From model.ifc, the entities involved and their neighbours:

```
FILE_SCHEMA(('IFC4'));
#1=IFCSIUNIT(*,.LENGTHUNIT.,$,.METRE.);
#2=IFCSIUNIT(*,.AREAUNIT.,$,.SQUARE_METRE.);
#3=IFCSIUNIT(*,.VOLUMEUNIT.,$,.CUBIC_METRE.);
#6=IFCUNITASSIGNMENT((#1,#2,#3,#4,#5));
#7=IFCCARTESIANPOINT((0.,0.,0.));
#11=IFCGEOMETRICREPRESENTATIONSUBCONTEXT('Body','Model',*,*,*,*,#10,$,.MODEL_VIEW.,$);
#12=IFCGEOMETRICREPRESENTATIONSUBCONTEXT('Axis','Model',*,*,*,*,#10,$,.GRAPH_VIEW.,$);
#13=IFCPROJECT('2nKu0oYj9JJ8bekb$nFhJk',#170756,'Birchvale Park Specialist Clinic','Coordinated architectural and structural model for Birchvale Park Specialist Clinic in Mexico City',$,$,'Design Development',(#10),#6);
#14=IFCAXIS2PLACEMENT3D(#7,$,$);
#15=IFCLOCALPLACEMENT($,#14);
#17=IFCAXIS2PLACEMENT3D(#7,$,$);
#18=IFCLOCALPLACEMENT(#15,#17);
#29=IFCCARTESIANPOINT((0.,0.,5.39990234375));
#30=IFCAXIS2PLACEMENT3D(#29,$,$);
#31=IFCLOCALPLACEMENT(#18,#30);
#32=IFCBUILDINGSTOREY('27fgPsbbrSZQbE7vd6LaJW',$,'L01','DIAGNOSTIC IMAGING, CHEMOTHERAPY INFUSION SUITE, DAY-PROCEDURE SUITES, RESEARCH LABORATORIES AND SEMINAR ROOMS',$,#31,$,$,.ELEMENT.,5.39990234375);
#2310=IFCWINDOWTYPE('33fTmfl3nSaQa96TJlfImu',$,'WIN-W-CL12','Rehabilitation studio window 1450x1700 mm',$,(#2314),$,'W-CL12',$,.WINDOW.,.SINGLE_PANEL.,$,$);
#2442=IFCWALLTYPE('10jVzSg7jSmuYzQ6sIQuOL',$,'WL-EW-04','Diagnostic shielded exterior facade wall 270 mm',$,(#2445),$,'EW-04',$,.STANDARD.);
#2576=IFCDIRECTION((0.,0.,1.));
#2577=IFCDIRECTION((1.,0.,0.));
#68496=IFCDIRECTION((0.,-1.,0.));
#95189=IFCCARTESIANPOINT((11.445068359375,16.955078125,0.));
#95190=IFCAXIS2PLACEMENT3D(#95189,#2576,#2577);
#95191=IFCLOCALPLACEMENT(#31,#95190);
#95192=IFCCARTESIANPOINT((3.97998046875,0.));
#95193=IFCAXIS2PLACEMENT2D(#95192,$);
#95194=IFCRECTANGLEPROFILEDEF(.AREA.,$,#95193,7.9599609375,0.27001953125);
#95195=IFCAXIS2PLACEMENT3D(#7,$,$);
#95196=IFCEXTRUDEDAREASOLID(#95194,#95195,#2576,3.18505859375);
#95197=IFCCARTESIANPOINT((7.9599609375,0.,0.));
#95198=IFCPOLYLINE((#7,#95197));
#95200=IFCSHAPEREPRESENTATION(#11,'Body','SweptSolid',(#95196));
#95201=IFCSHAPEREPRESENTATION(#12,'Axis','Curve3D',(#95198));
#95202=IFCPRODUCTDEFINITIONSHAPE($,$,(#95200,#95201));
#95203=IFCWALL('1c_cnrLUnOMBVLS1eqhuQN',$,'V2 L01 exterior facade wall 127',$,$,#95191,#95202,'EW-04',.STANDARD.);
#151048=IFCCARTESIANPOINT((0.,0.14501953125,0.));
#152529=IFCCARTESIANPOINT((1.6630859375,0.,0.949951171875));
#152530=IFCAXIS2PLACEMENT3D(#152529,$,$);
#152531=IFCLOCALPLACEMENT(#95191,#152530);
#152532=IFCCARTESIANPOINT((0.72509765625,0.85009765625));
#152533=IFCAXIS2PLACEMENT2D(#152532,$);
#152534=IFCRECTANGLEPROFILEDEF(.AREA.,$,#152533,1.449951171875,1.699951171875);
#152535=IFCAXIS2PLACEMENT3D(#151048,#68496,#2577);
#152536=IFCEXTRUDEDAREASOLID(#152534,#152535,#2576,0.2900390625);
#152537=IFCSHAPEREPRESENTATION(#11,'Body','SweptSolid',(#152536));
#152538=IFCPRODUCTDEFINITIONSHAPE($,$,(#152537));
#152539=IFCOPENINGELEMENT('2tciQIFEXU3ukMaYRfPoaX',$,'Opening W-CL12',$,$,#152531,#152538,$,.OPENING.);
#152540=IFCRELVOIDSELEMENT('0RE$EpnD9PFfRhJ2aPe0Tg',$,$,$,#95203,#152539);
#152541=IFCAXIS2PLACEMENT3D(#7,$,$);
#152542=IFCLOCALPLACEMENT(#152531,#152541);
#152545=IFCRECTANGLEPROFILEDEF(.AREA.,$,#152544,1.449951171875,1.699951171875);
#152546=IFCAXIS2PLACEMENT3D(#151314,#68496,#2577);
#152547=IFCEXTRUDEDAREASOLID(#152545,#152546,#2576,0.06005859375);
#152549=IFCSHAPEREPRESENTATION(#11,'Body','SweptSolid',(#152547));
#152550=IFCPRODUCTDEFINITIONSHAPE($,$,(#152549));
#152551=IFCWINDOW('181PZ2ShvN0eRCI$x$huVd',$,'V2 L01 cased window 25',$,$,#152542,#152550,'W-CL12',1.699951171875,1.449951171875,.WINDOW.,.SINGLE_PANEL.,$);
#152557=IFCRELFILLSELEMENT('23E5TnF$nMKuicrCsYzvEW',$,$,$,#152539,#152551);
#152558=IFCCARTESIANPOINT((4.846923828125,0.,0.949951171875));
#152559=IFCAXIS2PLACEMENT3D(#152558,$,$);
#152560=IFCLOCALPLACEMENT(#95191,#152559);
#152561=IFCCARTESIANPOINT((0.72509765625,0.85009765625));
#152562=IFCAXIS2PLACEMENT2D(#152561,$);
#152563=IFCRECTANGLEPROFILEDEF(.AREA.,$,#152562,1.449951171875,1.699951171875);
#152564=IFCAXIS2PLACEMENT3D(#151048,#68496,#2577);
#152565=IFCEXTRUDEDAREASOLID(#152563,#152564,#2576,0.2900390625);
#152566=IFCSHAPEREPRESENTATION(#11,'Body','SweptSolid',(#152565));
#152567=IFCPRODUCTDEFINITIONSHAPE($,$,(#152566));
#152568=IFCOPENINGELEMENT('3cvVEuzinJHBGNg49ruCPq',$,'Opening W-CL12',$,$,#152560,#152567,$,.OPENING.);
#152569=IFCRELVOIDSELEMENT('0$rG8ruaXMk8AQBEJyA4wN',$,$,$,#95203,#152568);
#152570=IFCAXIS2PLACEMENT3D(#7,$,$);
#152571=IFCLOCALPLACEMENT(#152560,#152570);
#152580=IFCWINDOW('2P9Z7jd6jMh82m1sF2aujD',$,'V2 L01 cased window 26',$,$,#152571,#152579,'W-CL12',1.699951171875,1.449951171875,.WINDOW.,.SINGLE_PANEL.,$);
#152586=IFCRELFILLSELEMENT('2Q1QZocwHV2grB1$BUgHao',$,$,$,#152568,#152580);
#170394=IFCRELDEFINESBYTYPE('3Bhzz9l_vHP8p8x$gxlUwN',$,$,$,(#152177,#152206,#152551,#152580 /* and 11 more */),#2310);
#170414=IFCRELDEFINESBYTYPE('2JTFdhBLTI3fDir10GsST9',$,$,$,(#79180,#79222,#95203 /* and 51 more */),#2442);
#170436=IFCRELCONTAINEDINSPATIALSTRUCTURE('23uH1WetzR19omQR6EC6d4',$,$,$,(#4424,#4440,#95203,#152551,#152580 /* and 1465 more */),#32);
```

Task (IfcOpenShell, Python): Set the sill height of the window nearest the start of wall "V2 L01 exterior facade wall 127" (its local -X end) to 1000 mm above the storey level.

```python
import numpy as np
import ifcopenshell
import ifcopenshell.api.geometry
import ifcopenshell.geom
import ifcopenshell.util.element
import ifcopenshell.util.placement
import ifcopenshell.util.shape
import ifcopenshell.util.unit

model = ifcopenshell.open("model.ifc")
unit_scale = ifcopenshell.util.unit.calculate_unit_scale(model)

window = model.by_id(152551)
opening = window.FillsVoids[0].RelatingOpeningElement
storey = ifcopenshell.util.element.get_container(window, ifc_class="IfcBuildingStorey")
level = ifcopenshell.util.placement.get_local_placement(storey.ObjectPlacement)[2, 3]

# The opening's origin need not be at the sill, so measure its lowest point.
shape = ifcopenshell.geom.create_shape(ifcopenshell.geom.settings(), opening)
bottom = ifcopenshell.util.shape.get_shape_bottom_elevation(shape, shape.geometry) / unit_scale
dz = level + 1 / unit_scale - bottom

shift = np.array([0.0, 0.0, dz])
# The window is placed relative to its opening, so it follows when the opening moves.
matrix = ifcopenshell.util.placement.get_local_placement(opening.ObjectPlacement)
matrix[:3, 3] += shift
ifcopenshell.api.geometry.edit_object_placement(
    model, product=opening, matrix=matrix, is_si=False, should_transform_children=True
)

print(f"moved by {dz * unit_scale:+.3f} m")

model.write("model_edited.ifc")
```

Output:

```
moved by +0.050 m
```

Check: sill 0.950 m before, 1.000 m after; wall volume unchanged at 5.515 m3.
